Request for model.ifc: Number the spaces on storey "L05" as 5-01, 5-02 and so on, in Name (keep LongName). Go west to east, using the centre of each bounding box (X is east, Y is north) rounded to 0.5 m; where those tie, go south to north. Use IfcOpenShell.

First a look at what the model holds.

```python
import ifcopenshell
import ifcopenshell.util.element
import ifcopenshell.util.placement

model = ifcopenshell.open("model.ifc")
print(model.schema)
storey = next(s for s in model.by_type("IfcBuildingStorey") if s.Name == "L05")
spaces = [e for e in ifcopenshell.util.element.get_decomposition(storey) if e.is_a("IfcSpace")]
for e in sorted(spaces, key=lambda e: e.id()):
    origin = ifcopenshell.util.placement.get_local_placement(e.ObjectPlacement)[:3, 3]
    print(e.id(), e.Name, e.LongName, origin.round(2) + 0.0, sep=" | ")
```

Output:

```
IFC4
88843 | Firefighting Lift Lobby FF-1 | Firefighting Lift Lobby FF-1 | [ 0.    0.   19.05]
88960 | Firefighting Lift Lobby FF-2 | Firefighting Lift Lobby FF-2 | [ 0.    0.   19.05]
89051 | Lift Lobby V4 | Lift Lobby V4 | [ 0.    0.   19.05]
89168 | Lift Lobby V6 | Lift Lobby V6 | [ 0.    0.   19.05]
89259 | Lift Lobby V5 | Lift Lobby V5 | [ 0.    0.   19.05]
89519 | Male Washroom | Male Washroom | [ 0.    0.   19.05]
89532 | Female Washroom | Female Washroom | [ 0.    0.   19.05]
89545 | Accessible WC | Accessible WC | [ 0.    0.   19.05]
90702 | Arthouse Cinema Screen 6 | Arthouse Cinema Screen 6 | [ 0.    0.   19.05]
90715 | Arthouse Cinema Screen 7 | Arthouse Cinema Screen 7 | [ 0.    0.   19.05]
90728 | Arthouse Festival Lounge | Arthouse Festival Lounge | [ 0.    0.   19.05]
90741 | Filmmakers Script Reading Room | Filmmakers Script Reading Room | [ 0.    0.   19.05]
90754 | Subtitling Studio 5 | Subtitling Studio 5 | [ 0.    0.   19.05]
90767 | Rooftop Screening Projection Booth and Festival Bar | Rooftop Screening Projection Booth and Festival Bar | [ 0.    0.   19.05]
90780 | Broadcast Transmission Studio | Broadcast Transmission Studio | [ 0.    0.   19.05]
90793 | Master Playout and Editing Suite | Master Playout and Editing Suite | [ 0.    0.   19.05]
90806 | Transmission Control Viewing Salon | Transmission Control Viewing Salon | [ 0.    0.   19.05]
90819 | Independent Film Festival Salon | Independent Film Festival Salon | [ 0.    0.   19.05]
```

```python
import ifcopenshell
import ifcopenshell.geom
import ifcopenshell.util.element
import ifcopenshell.util.shape

model = ifcopenshell.open("model.ifc")
settings = ifcopenshell.geom.settings()
settings.set("use-world-coords", True)


def centre(element):
    shape = ifcopenshell.geom.create_shape(settings, element)
    return ifcopenshell.util.shape.get_bbox_centroid(shape.geometry)


storey = next(s for s in model.by_type("IfcBuildingStorey") if s.Name == "L05")
spaces = [e for e in ifcopenshell.util.element.get_decomposition(storey) if e.is_a("IfcSpace")]

# Insertion points can sit at a corner or the storey origin, so sort by the geometry (in metres).
centres = {e: centre(e) for e in spaces}
spaces.sort(key=lambda e: (round(centres[e][0] / 0.5), centres[e][1]))

for i, e in enumerate(spaces, start=1):
    number = f"5-{i:02d}"
    e.Name = number
    print(e.id(), number)

model.write("model_rev.ifc")
```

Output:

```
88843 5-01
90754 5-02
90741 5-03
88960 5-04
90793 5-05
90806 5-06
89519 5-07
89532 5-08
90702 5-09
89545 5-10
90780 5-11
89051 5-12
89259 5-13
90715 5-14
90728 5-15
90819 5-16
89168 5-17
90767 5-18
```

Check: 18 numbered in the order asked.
